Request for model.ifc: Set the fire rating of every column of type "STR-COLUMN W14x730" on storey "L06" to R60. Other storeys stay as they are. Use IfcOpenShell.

First a look at what the model holds.

```python
import ifcopenshell
import ifcopenshell.util.element

model = ifcopenshell.open("model.ifc")
print(model.schema)
storey = next(s for s in model.by_type("IfcBuildingStorey") if s.Name == "L06")
columns = [e for e in ifcopenshell.util.element.get_decomposition(storey) if e.is_a("IfcColumn")]
seen = {}
for e in columns:
    element_type = ifcopenshell.util.element.get_type(e)
    key = (element_type.Name if element_type != e and element_type else None, ifcopenshell.util.element.get_pset(e, "Pset_ColumnCommon", "FireRating"))
    seen[key] = seen.get(key, 0) + 1
for (name, value), count in sorted(seen.items(), key=str):
    print(count, "x", name, "|", value)
```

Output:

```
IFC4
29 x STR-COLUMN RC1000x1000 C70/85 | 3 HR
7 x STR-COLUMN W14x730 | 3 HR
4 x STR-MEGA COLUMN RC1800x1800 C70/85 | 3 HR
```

```python
import ifcopenshell
import ifcopenshell.api.pset
import ifcopenshell.util.element

model = ifcopenshell.open("model.ifc")

storey = next(s for s in model.by_type("IfcBuildingStorey") if s.Name == "L06")
columns = [e for e in ifcopenshell.util.element.get_decomposition(storey) if e.is_a("IfcColumn")]

count = 0
for e in columns:
    element_type = ifcopenshell.util.element.get_type(e)
    if element_type in (None, e) or element_type.Name != "STR-COLUMN W14x730":
        continue
    found = ifcopenshell.util.element.get_pset(e, "Pset_ColumnCommon", should_inherit=False)
    if found:
        pset = model.by_id(found["id"])
        if len(ifcopenshell.util.element.get_elements_by_pset(pset)) > 1:
            pset = ifcopenshell.api.pset.unshare_pset(model, products=[e], pset=pset)[0]
    else:
        pset = ifcopenshell.api.pset.add_pset(model, product=e, name="Pset_ColumnCommon")
    ifcopenshell.api.pset.edit_pset(model, pset=pset, properties={"FireRating": "R60"})
    count += 1

print(count, "columns updated")

model.write("model_v2.ifc")
```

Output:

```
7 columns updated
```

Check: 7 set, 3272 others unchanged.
